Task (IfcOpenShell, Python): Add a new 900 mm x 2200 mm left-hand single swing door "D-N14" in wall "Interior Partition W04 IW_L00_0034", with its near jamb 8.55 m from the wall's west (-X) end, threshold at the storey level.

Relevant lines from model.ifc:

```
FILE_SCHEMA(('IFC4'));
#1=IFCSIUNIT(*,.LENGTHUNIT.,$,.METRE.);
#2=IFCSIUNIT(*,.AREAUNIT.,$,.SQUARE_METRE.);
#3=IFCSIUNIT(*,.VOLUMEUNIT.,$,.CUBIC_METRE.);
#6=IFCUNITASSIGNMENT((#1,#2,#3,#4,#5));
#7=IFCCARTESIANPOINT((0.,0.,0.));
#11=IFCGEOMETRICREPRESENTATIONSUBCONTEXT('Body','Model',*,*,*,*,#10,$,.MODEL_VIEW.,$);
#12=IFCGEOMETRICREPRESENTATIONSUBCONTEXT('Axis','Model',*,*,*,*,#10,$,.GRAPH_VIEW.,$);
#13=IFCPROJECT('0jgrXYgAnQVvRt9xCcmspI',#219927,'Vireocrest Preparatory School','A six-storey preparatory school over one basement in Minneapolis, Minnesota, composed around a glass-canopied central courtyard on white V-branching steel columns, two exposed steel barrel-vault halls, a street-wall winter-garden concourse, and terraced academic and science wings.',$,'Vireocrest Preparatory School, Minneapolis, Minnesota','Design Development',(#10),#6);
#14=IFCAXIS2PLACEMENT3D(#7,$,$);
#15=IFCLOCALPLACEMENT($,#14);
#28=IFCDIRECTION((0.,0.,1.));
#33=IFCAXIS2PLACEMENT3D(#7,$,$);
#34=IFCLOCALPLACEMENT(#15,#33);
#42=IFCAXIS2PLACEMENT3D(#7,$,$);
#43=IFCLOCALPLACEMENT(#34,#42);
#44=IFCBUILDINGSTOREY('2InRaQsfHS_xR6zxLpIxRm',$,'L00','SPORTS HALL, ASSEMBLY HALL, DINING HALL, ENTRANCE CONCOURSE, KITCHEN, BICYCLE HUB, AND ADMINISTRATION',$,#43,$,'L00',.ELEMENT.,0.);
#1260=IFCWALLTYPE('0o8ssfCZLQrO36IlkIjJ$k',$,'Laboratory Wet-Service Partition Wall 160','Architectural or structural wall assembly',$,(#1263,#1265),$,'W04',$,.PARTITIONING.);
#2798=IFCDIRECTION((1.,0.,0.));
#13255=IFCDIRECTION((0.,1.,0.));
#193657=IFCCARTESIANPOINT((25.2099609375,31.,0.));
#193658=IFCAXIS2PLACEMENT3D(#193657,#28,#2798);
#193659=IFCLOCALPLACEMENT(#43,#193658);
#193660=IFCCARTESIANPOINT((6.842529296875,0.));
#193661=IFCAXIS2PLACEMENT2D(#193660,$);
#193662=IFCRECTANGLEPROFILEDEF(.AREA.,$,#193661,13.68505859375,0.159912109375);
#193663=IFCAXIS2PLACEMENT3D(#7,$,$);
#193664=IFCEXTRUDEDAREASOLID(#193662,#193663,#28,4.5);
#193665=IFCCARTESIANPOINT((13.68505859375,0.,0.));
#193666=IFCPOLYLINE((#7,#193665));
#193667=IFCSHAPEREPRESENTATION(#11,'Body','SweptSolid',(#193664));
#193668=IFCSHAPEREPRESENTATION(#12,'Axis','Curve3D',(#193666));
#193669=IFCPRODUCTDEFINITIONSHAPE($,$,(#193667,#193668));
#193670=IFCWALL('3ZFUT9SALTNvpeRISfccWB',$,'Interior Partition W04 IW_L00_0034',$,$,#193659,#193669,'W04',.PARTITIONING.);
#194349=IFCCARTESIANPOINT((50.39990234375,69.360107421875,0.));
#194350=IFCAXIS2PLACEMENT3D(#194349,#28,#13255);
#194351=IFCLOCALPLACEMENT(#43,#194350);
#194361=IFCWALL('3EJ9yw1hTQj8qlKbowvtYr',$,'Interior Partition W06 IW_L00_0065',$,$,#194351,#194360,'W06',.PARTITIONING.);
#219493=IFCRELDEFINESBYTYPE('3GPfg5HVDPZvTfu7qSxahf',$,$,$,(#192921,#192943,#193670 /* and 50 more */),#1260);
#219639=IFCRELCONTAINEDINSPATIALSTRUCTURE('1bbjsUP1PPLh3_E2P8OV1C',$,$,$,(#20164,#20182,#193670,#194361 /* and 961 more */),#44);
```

```python
import numpy as np
import ifcopenshell
import ifcopenshell.api.feature
import ifcopenshell.api.geometry
import ifcopenshell.api.root
import ifcopenshell.api.spatial
import ifcopenshell.geom
import ifcopenshell.util.element
import ifcopenshell.util.placement
import ifcopenshell.util.representation
import ifcopenshell.util.shape
import ifcopenshell.util.unit

model = ifcopenshell.open("model.ifc")
unit_scale = ifcopenshell.util.unit.calculate_unit_scale(model)
settings = ifcopenshell.geom.settings()


def volume(element):
    """Net volume in cubic metres, openings subtracted."""
    shape = ifcopenshell.geom.create_shape(settings, element)
    return ifcopenshell.util.shape.get_volume(shape.geometry)


wall = model.by_id(193670)
storey = ifcopenshell.util.element.get_container(wall, ifc_class="IfcBuildingStorey")
context = ifcopenshell.util.representation.get_context(model, "Model", "Body", "MODEL_VIEW")
before = volume(wall)

width, height, from_end, sill = 0.9, 2.2, 8.55, 0.0  # metres

# The wall runs along its own X axis, and the end named is its -X end.
wall_shape = ifcopenshell.geom.create_shape(settings, wall)
x, y, z = ifcopenshell.util.shape.get_vertices(wall_shape.geometry).T
start = x.min() + from_end
face, thickness = float(y.min()), float(y.max() - y.min())
wall_matrix = ifcopenshell.util.placement.get_local_placement(wall.ObjectPlacement)
level = ifcopenshell.util.placement.get_local_placement(storey.ObjectPlacement)[2, 3]


def in_wall(x, y):
    """Placement at x, y metres in the wall's axes, at sill height."""
    matrix = wall_matrix.copy()
    matrix[:, 3] = wall_matrix @ np.array([x / unit_scale, y / unit_scale, 0.0, 1.0])
    matrix[2, 3] = level + sill / unit_scale
    return matrix


# Opening: a box that overshoots both wall faces by 50 mm.
opening = ifcopenshell.api.root.create_entity(model, ifc_class="IfcOpeningElement", predefined_type="OPENING")
box = ifcopenshell.api.geometry.add_wall_representation(
    model, context=context, length=width, height=height, thickness=thickness + 0.1
)
ifcopenshell.api.geometry.assign_representation(model, product=opening, representation=box)
ifcopenshell.api.geometry.edit_object_placement(model, product=opening, matrix=in_wall(start, face - 0.05), is_si=False)
ifcopenshell.api.feature.add_feature(model, feature=opening, element=wall)

door = ifcopenshell.api.root.create_entity(model, ifc_class="IfcDoor", name="D-N14", predefined_type="DOOR")
door.OverallWidth, door.OverallHeight = width / unit_scale, height / unit_scale
door.OperationType = "SINGLE_SWING_LEFT"
body = ifcopenshell.api.geometry.add_door_representation(
    model,
    context=context,
    overall_width=door.OverallWidth,
    overall_height=door.OverallHeight,
    operation_type="SINGLE_SWING_LEFT",
    lining_properties={"LiningDepth": thickness / unit_scale, "ThresholdDepth": thickness / unit_scale},
)
ifcopenshell.api.geometry.assign_representation(model, product=door, representation=body)
ifcopenshell.api.spatial.assign_container(model, products=[door], relating_structure=storey)
ifcopenshell.api.feature.add_filling(model, opening=opening, element=door)

# The lining spans the wall, so the door starts at the wall face.
ifcopenshell.api.geometry.edit_object_placement(model, product=door, matrix=in_wall(start, face), is_si=False)

after = volume(wall)

print(f"wall volume {before:.3f} -> {after:.3f} m3")

model.write("model_edited.ifc")
```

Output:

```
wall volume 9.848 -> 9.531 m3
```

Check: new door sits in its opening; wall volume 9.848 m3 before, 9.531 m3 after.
